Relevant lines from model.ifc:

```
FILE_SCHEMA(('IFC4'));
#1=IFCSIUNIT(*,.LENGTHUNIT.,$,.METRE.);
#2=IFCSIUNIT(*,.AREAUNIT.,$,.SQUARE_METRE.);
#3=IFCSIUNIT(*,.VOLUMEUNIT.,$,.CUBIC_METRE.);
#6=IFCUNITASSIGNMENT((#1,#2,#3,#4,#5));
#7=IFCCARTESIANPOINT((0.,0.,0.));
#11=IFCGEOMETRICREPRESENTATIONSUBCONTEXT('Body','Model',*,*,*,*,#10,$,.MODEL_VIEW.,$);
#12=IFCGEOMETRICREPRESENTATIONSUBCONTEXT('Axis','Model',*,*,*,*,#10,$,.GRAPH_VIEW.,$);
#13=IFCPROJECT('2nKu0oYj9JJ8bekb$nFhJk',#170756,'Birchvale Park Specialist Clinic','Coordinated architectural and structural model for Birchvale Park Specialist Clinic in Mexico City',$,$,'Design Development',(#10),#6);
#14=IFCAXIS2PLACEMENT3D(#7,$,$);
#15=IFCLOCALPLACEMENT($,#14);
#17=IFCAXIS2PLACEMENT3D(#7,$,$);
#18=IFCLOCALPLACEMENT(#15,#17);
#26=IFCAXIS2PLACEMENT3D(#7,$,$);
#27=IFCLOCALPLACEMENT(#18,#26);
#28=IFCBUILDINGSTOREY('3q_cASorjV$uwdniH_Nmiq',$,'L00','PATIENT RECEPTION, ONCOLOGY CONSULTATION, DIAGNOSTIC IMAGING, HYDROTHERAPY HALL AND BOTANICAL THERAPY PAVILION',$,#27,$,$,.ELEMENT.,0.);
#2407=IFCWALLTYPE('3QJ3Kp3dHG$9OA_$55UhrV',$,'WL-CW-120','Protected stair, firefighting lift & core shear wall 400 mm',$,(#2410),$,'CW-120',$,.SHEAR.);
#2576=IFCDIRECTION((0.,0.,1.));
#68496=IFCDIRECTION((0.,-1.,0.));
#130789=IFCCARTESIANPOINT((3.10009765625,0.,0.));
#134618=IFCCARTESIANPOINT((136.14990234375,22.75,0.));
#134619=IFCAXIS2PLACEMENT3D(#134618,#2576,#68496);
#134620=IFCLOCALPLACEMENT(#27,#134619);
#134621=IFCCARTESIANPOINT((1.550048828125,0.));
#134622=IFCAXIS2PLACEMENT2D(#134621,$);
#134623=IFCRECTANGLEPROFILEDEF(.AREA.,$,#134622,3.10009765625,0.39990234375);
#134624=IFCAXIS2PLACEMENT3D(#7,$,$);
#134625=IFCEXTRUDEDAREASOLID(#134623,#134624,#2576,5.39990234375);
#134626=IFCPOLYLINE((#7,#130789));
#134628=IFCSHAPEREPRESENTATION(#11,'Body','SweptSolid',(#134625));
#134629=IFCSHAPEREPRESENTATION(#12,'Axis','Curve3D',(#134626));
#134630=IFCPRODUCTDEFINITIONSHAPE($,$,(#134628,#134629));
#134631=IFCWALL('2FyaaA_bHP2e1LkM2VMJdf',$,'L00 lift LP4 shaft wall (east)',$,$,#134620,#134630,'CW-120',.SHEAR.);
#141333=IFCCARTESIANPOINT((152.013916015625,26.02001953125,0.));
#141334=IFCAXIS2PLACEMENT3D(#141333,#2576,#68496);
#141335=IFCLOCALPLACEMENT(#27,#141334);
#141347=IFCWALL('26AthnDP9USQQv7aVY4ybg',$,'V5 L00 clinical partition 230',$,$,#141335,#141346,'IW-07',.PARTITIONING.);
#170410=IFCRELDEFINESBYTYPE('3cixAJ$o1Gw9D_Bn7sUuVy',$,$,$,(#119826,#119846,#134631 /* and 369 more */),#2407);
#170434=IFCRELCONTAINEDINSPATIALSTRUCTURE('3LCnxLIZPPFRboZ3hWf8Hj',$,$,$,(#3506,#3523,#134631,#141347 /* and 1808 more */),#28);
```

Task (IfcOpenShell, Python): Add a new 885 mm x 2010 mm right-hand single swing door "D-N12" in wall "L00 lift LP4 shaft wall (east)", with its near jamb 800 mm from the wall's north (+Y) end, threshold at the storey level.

```python
import numpy as np
import ifcopenshell
import ifcopenshell.api.feature
import ifcopenshell.api.geometry
import ifcopenshell.api.root
import ifcopenshell.api.spatial
import ifcopenshell.geom
import ifcopenshell.util.element
import ifcopenshell.util.placement
import ifcopenshell.util.representation
import ifcopenshell.util.shape
import ifcopenshell.util.unit

model = ifcopenshell.open("model.ifc")
unit_scale = ifcopenshell.util.unit.calculate_unit_scale(model)
settings = ifcopenshell.geom.settings()


def volume(element):
    """Net volume in cubic metres, openings subtracted."""
    shape = ifcopenshell.geom.create_shape(settings, element)
    return ifcopenshell.util.shape.get_volume(shape.geometry)


wall = model.by_id(134631)
storey = ifcopenshell.util.element.get_container(wall, ifc_class="IfcBuildingStorey")
context = ifcopenshell.util.representation.get_context(model, "Model", "Body", "MODEL_VIEW")
before = volume(wall)

width, height, from_end, sill = 0.885, 2.01, 0.8, 0.0  # metres

# The wall runs along its own X axis, and the end named is its -X end.
wall_shape = ifcopenshell.geom.create_shape(settings, wall)
x, y, z = ifcopenshell.util.shape.get_vertices(wall_shape.geometry).T
start = x.min() + from_end
face, thickness = float(y.min()), float(y.max() - y.min())
wall_matrix = ifcopenshell.util.placement.get_local_placement(wall.ObjectPlacement)
level = ifcopenshell.util.placement.get_local_placement(storey.ObjectPlacement)[2, 3]


def in_wall(x, y):
    """Placement at x, y metres in the wall's axes, at sill height."""
    matrix = wall_matrix.copy()
    matrix[:, 3] = wall_matrix @ np.array([x / unit_scale, y / unit_scale, 0.0, 1.0])
    matrix[2, 3] = level + sill / unit_scale
    return matrix


# Opening: a box that overshoots both wall faces by 50 mm.
opening = ifcopenshell.api.root.create_entity(model, ifc_class="IfcOpeningElement", predefined_type="OPENING")
box = ifcopenshell.api.geometry.add_wall_representation(
    model, context=context, length=width, height=height, thickness=thickness + 0.1
)
ifcopenshell.api.geometry.assign_representation(model, product=opening, representation=box)
ifcopenshell.api.geometry.edit_object_placement(model, product=opening, matrix=in_wall(start, face - 0.05), is_si=False)
ifcopenshell.api.feature.add_feature(model, feature=opening, element=wall)

door = ifcopenshell.api.root.create_entity(model, ifc_class="IfcDoor", name="D-N12", predefined_type="DOOR")
door.OverallWidth, door.OverallHeight = width / unit_scale, height / unit_scale
door.OperationType = "SINGLE_SWING_RIGHT"
body = ifcopenshell.api.geometry.add_door_representation(
    model,
    context=context,
    overall_width=door.OverallWidth,
    overall_height=door.OverallHeight,
    operation_type="SINGLE_SWING_RIGHT",
    lining_properties={"LiningDepth": thickness / unit_scale, "ThresholdDepth": thickness / unit_scale},
)
ifcopenshell.api.geometry.assign_representation(model, product=door, representation=body)
ifcopenshell.api.spatial.assign_container(model, products=[door], relating_structure=storey)
ifcopenshell.api.feature.add_filling(model, opening=opening, element=door)

# The lining spans the wall, so the door starts at the wall face.
ifcopenshell.api.geometry.edit_object_placement(model, product=door, matrix=in_wall(start, face), is_si=False)

after = volume(wall)

print(f"wall volume {before:.3f} -> {after:.3f} m3")

model.write("model_updated.ifc")
```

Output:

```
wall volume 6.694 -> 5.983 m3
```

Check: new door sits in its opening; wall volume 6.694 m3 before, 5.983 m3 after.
